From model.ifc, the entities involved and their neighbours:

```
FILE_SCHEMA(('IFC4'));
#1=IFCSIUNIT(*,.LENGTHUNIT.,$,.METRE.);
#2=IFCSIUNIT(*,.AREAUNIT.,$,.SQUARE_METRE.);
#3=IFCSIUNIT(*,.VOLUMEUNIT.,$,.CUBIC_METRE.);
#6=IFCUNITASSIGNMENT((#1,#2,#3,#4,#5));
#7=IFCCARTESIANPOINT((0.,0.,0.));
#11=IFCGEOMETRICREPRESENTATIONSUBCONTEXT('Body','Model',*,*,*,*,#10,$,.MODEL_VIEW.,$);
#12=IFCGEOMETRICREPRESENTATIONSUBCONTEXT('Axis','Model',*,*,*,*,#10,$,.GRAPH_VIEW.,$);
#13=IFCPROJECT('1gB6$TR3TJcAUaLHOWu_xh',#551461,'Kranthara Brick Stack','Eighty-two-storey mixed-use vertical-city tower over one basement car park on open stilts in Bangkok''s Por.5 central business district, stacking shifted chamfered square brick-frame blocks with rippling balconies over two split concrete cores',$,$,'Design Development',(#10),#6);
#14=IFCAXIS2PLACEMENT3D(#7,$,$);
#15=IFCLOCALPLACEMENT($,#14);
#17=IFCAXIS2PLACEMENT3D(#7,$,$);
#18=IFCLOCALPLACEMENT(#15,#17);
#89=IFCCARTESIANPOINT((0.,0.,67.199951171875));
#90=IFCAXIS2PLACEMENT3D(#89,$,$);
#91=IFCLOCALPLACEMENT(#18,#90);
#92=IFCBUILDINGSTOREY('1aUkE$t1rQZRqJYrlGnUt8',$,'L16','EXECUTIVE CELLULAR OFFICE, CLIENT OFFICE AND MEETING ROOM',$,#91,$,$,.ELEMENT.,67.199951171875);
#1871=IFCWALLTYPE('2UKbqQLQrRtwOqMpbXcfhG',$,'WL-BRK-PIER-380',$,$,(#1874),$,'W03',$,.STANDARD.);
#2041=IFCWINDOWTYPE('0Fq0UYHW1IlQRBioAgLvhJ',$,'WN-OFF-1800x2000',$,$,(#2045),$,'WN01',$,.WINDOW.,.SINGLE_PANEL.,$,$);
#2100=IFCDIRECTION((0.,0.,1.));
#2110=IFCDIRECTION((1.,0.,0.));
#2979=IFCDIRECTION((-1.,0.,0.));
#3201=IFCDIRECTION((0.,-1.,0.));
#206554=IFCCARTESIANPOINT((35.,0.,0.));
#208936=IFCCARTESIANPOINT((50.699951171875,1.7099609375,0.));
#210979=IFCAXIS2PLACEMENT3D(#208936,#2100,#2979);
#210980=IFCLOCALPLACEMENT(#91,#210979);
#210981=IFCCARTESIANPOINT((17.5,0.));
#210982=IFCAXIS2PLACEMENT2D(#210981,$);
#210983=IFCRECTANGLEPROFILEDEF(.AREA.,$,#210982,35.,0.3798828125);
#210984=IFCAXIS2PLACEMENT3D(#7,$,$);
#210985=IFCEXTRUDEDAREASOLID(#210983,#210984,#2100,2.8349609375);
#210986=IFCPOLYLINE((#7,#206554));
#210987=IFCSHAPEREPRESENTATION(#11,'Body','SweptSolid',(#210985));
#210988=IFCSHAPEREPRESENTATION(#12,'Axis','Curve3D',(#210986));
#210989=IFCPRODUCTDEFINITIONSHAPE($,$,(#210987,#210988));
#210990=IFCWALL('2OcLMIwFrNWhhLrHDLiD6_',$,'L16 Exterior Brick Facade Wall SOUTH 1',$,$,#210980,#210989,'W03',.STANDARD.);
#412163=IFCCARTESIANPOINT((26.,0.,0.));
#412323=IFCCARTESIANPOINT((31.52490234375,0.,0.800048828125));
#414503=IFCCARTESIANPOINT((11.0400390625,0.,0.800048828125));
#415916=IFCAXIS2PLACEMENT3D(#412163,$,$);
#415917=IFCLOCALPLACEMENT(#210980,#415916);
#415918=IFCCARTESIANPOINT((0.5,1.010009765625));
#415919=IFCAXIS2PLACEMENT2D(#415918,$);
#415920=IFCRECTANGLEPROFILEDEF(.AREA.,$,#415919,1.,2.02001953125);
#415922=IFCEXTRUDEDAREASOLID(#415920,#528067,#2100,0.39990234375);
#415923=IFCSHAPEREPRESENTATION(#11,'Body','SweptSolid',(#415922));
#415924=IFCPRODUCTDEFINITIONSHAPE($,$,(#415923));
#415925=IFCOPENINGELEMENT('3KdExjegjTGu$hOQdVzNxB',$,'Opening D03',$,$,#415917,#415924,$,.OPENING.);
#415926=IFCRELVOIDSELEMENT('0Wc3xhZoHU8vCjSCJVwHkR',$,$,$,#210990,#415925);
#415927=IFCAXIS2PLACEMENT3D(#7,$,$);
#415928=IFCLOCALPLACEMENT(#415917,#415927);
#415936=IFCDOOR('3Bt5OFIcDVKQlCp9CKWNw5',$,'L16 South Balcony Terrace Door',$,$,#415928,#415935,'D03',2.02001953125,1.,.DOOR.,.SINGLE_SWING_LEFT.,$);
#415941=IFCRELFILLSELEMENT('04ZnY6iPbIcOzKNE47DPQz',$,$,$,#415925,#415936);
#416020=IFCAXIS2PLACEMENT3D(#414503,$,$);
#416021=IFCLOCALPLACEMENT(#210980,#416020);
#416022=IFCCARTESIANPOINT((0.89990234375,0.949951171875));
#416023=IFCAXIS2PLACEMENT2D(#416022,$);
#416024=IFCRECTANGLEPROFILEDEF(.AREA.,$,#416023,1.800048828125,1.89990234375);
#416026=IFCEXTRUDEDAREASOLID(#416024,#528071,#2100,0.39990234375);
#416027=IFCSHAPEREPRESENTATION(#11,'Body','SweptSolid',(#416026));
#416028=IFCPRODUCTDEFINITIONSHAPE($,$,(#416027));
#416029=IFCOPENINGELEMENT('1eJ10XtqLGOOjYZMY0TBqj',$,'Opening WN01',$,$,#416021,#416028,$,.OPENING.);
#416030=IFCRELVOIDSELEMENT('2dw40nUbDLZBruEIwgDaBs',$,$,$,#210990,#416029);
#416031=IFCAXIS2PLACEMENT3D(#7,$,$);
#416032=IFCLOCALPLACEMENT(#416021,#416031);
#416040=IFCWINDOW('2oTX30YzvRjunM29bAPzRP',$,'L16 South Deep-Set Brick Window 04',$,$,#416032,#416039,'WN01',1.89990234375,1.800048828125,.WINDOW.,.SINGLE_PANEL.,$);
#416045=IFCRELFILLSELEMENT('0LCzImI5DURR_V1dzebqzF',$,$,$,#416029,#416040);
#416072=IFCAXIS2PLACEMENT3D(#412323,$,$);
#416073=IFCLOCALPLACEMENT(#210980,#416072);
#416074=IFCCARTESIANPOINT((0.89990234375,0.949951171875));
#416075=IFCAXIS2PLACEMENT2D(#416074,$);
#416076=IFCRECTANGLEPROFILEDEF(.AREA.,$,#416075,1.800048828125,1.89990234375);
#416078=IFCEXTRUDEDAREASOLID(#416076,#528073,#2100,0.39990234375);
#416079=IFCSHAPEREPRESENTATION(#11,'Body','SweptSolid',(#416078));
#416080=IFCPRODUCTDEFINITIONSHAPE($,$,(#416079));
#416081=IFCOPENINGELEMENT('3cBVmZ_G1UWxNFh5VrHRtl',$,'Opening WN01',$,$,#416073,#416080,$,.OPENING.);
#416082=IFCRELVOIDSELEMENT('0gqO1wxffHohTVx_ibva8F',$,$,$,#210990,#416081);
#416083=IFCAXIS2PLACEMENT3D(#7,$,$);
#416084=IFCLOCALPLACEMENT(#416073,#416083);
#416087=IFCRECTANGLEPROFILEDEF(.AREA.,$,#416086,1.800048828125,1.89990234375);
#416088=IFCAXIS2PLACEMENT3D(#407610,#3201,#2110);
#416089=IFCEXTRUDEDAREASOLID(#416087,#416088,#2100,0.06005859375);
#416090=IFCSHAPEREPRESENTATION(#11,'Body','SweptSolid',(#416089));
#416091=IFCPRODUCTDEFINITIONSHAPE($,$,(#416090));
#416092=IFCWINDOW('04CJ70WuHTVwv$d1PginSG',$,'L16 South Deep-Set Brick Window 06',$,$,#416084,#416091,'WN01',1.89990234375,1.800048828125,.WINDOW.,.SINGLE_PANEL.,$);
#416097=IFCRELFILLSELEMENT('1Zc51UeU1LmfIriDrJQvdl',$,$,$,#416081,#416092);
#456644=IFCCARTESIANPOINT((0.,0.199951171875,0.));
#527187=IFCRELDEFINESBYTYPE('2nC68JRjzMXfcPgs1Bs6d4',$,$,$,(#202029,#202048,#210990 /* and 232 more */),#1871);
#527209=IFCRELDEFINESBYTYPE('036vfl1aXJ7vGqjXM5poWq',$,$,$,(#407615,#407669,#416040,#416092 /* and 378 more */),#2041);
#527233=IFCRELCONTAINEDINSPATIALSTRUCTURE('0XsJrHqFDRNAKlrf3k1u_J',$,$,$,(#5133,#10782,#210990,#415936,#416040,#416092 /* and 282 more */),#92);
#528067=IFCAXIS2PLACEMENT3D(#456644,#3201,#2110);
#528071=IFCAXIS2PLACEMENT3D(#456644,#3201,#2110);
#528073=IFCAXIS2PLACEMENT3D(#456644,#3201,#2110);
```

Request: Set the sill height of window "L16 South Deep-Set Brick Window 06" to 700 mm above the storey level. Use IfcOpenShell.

```python
import numpy as np
import ifcopenshell
import ifcopenshell.api.geometry
import ifcopenshell.geom
import ifcopenshell.util.element
import ifcopenshell.util.placement
import ifcopenshell.util.shape
import ifcopenshell.util.unit

model = ifcopenshell.open("model.ifc")
unit_scale = ifcopenshell.util.unit.calculate_unit_scale(model)

window = model.by_guid("04CJ70WuHTVwv$d1PginSG")
opening = window.FillsVoids[0].RelatingOpeningElement
storey = ifcopenshell.util.element.get_container(window, ifc_class="IfcBuildingStorey")
level = ifcopenshell.util.placement.get_local_placement(storey.ObjectPlacement)[2, 3]

# The opening's origin need not be at the sill, so measure its lowest point.
shape = ifcopenshell.geom.create_shape(ifcopenshell.geom.settings(), opening)
bottom = ifcopenshell.util.shape.get_shape_bottom_elevation(shape, shape.geometry) / unit_scale
dz = level + 0.7 - bottom

shift = np.array([0.0, 0.0, dz])
# The window is placed relative to its opening, so it follows when the opening moves.
matrix = ifcopenshell.util.placement.get_local_placement(opening.ObjectPlacement)
matrix[:3, 3] += shift
ifcopenshell.api.geometry.edit_object_placement(
    model, product=opening, matrix=matrix, is_si=False, should_transform_children=True
)

print(f"moved by {dz * unit_scale:+.3f} m")

model.write("model_rev.ifc")
```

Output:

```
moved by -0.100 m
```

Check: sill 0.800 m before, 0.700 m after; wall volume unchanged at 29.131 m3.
